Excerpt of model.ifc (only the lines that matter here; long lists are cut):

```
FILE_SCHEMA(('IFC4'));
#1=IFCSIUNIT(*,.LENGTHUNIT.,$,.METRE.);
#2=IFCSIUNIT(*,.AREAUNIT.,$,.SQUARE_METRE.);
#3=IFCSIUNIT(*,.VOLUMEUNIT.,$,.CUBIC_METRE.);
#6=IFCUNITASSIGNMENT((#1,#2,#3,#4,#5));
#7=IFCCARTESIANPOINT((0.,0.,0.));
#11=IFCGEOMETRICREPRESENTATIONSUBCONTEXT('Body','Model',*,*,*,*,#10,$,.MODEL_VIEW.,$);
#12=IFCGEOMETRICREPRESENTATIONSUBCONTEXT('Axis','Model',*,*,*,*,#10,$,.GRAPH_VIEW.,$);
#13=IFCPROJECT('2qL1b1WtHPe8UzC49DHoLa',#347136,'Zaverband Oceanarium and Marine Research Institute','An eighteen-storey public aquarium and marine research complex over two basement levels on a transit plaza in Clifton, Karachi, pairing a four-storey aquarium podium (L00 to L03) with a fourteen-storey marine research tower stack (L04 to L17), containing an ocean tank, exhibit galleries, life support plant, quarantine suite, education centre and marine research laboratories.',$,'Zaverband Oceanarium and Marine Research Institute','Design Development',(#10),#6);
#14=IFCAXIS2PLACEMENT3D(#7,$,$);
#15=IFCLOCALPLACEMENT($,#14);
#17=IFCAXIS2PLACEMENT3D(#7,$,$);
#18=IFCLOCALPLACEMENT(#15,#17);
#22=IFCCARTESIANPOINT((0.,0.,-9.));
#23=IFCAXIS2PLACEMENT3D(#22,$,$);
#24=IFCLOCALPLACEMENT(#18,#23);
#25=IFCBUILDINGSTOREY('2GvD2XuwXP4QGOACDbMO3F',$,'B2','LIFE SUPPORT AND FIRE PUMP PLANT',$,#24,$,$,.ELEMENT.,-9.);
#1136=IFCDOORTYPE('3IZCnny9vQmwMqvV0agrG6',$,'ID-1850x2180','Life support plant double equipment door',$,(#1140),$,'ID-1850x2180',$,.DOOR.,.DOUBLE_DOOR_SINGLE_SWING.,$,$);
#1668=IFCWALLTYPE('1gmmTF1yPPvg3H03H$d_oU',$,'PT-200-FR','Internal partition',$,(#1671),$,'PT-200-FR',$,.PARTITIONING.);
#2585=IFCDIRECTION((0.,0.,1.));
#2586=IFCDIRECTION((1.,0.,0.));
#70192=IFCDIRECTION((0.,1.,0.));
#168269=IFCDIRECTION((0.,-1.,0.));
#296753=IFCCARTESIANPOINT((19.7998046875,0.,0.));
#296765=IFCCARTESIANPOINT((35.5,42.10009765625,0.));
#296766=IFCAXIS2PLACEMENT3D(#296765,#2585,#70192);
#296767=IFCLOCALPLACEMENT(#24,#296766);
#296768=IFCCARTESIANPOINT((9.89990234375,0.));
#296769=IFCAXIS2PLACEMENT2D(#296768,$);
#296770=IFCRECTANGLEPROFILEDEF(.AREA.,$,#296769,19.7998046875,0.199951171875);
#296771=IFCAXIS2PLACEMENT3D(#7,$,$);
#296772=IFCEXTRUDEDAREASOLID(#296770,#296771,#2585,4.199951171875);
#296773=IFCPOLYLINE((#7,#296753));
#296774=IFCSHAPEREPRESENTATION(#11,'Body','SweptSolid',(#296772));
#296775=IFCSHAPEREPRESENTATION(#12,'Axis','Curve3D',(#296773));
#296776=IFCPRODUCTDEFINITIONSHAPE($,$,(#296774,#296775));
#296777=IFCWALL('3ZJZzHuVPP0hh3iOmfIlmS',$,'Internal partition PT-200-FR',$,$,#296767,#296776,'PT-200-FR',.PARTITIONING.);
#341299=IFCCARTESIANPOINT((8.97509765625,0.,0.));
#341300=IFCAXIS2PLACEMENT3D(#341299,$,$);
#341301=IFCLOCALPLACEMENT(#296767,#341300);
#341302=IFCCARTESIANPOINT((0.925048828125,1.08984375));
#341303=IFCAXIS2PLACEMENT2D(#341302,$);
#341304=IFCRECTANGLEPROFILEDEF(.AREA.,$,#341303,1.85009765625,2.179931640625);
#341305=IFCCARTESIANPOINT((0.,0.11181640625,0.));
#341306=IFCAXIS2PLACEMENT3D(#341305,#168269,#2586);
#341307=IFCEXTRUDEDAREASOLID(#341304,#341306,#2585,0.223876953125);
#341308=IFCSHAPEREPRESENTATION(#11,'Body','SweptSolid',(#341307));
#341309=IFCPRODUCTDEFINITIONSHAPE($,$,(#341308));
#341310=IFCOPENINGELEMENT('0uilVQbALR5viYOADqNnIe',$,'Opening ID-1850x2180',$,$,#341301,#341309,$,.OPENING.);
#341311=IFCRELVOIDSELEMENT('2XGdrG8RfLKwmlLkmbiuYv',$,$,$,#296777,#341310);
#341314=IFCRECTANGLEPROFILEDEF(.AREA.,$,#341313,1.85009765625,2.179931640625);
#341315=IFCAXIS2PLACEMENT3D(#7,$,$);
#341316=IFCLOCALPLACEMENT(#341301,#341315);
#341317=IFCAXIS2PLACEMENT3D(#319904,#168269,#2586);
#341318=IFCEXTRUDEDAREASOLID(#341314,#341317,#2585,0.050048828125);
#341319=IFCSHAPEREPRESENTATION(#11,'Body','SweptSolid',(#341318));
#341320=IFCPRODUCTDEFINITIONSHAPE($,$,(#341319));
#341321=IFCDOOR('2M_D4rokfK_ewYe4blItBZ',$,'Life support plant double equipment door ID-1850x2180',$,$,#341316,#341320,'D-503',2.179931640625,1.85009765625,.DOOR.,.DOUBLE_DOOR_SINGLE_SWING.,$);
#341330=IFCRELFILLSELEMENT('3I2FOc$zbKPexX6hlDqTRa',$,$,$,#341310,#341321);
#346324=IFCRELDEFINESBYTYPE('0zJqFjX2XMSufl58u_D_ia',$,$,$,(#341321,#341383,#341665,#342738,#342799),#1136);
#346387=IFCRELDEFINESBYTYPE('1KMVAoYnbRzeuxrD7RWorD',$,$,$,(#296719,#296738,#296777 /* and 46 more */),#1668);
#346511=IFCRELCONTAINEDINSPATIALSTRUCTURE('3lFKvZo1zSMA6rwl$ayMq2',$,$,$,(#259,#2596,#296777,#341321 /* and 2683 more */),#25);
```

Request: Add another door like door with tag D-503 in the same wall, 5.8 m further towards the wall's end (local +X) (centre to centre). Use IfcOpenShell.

```python
import ifcopenshell
import ifcopenshell.api.feature
import ifcopenshell.api.geometry
import ifcopenshell.api.root
import ifcopenshell.geom
import ifcopenshell.util.element
import ifcopenshell.util.placement
import ifcopenshell.util.shape
import ifcopenshell.util.unit

model = ifcopenshell.open("model.ifc")
unit_scale = ifcopenshell.util.unit.calculate_unit_scale(model)
settings = ifcopenshell.geom.settings()


def volume(element):
    """Net volume in cubic metres, openings subtracted."""
    shape = ifcopenshell.geom.create_shape(settings, element)
    return ifcopenshell.util.shape.get_volume(shape.geometry)


door = model.by_guid("2M_D4rokfK_ewYe4blItBZ")
opening = door.FillsVoids[0].RelatingOpeningElement
wall = opening.VoidsElements[0].RelatingBuildingElement
before = volume(wall)
shift = ifcopenshell.util.placement.get_local_placement(wall.ObjectPlacement)[:3, 0] * 5.8 / unit_scale

# copy_class copies the void relationship, type, container and properties, but no geometry.
new_opening = ifcopenshell.api.root.copy_class(model, product=opening)
new_opening.Representation = ifcopenshell.util.element.copy_deep(
    model, opening.Representation, exclude=["IfcGeometricRepresentationContext", "IfcRepresentationMap"]
)
new_door = ifcopenshell.api.root.copy_class(model, product=door)
new_door.Representation = ifcopenshell.util.element.copy_deep(
    model, door.Representation, exclude=["IfcGeometricRepresentationContext", "IfcRepresentationMap"]
)
new_door.Tag = None
ifcopenshell.api.feature.add_filling(model, opening=new_opening, element=new_door)

for old, new in ((opening, new_opening), (door, new_door)):
    matrix = ifcopenshell.util.placement.get_local_placement(old.ObjectPlacement)
    matrix[:3, 3] += shift
    ifcopenshell.api.geometry.edit_object_placement(model, product=new, matrix=matrix, is_si=False)

after = volume(wall)

print(f"wall volume {before:.3f} -> {after:.3f} m3")

model.write("model_updated.ifc")
```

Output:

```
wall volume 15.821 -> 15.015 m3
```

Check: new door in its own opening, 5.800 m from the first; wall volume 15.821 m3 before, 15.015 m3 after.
